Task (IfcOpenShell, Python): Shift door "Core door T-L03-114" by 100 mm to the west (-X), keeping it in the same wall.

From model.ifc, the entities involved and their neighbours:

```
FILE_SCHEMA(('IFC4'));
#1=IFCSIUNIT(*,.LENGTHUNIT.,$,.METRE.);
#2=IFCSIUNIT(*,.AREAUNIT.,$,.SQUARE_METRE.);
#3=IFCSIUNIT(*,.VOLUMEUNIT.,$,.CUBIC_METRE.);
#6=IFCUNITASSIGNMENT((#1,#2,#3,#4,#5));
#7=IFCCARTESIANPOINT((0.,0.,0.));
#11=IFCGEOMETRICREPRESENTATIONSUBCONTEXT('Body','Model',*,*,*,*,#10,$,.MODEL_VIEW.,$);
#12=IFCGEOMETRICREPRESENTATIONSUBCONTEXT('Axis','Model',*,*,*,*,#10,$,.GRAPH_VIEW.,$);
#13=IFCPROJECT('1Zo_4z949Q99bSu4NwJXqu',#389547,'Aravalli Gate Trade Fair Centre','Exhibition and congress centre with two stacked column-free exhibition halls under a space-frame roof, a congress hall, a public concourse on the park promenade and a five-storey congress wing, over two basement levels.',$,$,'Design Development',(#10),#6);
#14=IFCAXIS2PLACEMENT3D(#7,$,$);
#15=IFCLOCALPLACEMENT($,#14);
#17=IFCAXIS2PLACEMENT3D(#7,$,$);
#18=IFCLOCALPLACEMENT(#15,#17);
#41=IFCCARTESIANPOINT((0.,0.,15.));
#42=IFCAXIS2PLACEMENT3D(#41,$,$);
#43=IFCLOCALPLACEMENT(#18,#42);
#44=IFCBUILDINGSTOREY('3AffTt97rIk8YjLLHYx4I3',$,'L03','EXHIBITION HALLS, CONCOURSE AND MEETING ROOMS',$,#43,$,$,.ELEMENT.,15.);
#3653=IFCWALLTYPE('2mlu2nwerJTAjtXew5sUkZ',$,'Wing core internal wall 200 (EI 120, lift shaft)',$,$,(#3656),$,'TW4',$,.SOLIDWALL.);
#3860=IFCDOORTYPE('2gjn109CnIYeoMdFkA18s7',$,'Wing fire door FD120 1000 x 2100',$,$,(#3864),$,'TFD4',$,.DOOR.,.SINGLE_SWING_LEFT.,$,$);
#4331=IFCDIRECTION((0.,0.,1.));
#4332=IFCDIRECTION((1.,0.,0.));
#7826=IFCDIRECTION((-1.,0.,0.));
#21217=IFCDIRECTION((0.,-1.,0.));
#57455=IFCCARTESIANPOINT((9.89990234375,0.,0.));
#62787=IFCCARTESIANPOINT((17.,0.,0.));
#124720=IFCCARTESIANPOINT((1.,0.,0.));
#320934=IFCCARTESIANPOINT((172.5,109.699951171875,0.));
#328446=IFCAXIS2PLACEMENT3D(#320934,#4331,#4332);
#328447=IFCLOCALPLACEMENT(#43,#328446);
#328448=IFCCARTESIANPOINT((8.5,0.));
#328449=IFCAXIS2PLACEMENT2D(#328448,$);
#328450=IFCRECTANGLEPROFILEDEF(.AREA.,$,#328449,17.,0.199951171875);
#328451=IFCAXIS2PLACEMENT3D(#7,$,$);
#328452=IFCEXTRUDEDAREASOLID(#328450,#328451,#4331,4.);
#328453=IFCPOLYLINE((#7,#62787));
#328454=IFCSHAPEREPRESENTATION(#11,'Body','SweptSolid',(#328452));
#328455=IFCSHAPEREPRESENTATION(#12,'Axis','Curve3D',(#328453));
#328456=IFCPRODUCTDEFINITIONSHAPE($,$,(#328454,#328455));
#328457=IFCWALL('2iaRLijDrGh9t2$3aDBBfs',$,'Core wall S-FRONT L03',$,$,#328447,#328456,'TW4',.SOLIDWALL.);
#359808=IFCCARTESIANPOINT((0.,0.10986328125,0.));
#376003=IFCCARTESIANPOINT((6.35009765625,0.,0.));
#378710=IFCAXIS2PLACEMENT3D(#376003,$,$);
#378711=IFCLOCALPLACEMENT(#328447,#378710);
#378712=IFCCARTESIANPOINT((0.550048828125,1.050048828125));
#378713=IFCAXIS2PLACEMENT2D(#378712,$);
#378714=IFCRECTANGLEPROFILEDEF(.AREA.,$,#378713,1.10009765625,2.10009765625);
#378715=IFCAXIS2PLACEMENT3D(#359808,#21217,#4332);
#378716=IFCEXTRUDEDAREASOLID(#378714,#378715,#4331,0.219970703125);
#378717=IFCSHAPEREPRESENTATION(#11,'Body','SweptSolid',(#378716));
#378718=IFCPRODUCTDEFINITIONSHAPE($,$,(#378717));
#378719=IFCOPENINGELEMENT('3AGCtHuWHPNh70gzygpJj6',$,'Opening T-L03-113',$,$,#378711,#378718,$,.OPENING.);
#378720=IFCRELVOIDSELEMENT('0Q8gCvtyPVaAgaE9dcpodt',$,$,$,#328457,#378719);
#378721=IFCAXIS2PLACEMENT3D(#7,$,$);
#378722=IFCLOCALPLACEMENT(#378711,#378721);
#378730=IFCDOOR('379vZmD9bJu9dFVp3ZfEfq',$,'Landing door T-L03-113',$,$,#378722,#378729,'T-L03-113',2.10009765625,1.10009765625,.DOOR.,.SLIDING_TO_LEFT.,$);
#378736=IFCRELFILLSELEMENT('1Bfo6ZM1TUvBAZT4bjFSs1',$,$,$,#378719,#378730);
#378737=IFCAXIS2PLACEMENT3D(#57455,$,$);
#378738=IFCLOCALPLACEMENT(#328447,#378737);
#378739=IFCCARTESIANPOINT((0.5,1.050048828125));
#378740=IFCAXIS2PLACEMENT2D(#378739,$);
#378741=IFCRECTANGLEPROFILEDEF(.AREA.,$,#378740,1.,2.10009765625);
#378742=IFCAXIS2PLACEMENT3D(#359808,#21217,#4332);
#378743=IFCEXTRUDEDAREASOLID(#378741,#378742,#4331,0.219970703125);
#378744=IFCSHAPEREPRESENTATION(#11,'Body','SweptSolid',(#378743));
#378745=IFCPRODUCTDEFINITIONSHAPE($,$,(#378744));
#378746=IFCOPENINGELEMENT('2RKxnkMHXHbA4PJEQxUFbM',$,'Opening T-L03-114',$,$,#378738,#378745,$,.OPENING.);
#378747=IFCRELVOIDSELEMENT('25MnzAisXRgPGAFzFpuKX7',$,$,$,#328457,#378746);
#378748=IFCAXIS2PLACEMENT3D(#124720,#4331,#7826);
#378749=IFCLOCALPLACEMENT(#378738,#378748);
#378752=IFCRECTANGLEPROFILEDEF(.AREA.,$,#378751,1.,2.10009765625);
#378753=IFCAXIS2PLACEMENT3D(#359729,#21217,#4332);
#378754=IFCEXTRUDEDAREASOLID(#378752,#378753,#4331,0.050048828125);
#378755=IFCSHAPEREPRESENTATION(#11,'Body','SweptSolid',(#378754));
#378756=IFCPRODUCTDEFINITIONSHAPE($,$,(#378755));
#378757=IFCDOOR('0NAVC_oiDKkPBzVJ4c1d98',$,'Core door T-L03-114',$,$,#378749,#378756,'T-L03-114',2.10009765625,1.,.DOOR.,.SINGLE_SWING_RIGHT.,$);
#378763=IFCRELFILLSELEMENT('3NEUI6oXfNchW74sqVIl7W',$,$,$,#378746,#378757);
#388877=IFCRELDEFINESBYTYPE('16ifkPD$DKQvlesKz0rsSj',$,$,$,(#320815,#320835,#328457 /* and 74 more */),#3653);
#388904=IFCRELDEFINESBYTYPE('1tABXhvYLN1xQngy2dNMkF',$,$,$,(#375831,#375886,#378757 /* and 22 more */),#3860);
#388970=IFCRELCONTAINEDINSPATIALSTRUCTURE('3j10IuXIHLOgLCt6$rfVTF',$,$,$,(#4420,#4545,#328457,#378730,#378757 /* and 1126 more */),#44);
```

```python
import ifcopenshell
import ifcopenshell.api.geometry
import ifcopenshell.util.placement
import ifcopenshell.util.unit

model = ifcopenshell.open("model.ifc")
unit_scale = ifcopenshell.util.unit.calculate_unit_scale(model)

door = model.by_id(378757)
opening = door.FillsVoids[0].RelatingOpeningElement
wall = opening.VoidsElements[0].RelatingBuildingElement

wall_matrix = ifcopenshell.util.placement.get_local_placement(wall.ObjectPlacement)
shift = wall_matrix[:3, 0] * -0.1 / unit_scale
before = ifcopenshell.util.placement.get_local_placement(door.ObjectPlacement)[:3, 3].copy()

# The door is placed relative to its opening, so it follows when the opening moves.
matrix = ifcopenshell.util.placement.get_local_placement(opening.ObjectPlacement)
matrix[:3, 3] += shift
ifcopenshell.api.geometry.edit_object_placement(
    model, product=opening, matrix=matrix, is_si=False, should_transform_children=True
)

after = ifcopenshell.util.placement.get_local_placement(door.ObjectPlacement)[:3, 3]
print("door moved by", (after - before).round(3) + 0.0)

model.write("model_edited.ifc")
```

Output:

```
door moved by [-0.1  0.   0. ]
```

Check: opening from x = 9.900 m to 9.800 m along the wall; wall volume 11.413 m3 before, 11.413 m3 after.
